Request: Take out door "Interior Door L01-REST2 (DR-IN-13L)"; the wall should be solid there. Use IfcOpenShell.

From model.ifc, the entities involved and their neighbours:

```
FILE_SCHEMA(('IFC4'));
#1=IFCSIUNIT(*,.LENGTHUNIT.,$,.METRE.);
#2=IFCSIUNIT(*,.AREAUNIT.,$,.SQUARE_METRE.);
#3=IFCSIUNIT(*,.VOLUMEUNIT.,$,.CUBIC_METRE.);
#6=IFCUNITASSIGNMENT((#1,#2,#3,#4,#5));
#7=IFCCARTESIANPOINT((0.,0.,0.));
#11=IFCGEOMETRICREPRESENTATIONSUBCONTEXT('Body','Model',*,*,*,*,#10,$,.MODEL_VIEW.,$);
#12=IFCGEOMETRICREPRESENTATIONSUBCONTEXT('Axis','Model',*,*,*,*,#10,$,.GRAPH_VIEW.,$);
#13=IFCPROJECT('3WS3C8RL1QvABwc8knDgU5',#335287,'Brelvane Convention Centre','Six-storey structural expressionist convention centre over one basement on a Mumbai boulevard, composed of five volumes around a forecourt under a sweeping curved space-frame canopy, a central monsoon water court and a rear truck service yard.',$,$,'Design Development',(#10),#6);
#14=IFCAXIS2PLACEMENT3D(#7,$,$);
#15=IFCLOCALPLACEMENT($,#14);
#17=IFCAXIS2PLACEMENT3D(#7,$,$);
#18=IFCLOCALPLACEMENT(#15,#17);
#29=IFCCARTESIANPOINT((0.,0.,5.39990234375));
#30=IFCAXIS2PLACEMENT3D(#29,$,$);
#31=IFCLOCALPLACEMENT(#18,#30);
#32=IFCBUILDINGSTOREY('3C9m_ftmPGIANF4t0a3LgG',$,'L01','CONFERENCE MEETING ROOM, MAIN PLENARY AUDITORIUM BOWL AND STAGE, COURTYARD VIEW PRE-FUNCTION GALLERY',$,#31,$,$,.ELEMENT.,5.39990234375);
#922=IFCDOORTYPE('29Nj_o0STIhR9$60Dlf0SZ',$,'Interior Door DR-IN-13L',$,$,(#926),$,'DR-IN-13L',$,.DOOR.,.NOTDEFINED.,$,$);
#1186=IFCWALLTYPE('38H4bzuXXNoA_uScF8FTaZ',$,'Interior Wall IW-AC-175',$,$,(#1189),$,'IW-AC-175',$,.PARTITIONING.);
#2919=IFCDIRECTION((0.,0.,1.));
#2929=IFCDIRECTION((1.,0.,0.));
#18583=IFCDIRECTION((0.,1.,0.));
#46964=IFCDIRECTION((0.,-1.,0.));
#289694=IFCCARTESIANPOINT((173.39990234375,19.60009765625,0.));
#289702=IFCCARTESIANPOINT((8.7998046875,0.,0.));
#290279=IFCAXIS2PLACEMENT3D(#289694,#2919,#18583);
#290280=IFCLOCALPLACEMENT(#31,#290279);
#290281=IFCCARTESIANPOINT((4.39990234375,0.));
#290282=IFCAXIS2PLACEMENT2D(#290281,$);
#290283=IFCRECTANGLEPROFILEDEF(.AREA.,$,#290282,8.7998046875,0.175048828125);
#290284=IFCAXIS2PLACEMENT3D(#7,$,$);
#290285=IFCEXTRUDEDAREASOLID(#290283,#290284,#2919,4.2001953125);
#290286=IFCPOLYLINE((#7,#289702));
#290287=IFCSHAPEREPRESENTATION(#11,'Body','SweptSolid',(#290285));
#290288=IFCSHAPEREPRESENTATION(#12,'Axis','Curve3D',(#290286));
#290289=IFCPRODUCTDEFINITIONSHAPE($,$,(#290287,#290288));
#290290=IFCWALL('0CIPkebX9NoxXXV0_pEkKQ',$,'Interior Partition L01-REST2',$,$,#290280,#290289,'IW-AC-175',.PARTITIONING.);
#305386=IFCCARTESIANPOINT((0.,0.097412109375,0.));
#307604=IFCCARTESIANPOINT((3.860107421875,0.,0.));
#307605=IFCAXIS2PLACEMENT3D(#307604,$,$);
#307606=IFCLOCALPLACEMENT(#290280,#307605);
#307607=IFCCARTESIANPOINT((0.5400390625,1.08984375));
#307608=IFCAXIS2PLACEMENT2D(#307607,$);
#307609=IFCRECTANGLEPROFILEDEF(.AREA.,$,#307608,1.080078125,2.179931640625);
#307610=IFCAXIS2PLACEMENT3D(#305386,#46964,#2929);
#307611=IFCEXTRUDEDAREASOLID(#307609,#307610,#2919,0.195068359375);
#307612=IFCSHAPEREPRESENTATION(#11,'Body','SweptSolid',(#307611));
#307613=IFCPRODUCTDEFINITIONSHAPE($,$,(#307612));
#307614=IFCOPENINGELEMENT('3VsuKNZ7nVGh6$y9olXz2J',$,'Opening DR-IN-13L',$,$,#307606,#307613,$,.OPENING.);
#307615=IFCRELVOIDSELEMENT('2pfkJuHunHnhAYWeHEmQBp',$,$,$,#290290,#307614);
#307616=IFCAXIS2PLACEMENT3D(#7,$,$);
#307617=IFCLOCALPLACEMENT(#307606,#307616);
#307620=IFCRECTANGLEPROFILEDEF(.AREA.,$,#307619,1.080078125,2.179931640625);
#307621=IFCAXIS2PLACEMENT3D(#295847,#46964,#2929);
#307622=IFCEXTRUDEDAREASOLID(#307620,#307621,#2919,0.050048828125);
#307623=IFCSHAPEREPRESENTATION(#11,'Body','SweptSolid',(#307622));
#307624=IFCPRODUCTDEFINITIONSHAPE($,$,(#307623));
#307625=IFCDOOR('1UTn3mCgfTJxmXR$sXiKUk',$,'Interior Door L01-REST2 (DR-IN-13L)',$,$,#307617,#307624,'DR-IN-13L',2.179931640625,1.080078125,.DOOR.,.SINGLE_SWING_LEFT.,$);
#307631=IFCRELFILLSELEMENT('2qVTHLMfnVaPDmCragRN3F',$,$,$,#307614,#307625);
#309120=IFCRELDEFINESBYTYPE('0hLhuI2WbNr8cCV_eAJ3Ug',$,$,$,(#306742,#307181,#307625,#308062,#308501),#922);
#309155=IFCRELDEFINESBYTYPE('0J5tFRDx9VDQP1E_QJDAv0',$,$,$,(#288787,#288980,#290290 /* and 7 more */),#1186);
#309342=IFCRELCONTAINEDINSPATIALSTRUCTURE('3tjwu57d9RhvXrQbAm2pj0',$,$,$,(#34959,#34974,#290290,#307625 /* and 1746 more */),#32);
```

```python
import ifcopenshell
import ifcopenshell.api.feature
import ifcopenshell.api.root
import ifcopenshell.geom
import ifcopenshell.util.shape

model = ifcopenshell.open("model.ifc")
settings = ifcopenshell.geom.settings()


def volume(element):
    """Net volume in cubic metres, openings subtracted."""
    shape = ifcopenshell.geom.create_shape(settings, element)
    return ifcopenshell.util.shape.get_volume(shape.geometry)


door = model.by_id(307625)
opening = door.FillsVoids[0].RelatingOpeningElement
wall = opening.VoidsElements[0].RelatingBuildingElement
before = volume(wall)

ifcopenshell.api.root.remove_product(model, product=door)
ifcopenshell.api.feature.remove_feature(model, feature=opening)

after = volume(wall)

print(f"wall volume {before:.3f} -> {after:.3f} m3")

model.write("model_edited.ifc")
```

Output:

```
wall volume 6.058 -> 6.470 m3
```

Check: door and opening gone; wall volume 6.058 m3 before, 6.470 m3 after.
